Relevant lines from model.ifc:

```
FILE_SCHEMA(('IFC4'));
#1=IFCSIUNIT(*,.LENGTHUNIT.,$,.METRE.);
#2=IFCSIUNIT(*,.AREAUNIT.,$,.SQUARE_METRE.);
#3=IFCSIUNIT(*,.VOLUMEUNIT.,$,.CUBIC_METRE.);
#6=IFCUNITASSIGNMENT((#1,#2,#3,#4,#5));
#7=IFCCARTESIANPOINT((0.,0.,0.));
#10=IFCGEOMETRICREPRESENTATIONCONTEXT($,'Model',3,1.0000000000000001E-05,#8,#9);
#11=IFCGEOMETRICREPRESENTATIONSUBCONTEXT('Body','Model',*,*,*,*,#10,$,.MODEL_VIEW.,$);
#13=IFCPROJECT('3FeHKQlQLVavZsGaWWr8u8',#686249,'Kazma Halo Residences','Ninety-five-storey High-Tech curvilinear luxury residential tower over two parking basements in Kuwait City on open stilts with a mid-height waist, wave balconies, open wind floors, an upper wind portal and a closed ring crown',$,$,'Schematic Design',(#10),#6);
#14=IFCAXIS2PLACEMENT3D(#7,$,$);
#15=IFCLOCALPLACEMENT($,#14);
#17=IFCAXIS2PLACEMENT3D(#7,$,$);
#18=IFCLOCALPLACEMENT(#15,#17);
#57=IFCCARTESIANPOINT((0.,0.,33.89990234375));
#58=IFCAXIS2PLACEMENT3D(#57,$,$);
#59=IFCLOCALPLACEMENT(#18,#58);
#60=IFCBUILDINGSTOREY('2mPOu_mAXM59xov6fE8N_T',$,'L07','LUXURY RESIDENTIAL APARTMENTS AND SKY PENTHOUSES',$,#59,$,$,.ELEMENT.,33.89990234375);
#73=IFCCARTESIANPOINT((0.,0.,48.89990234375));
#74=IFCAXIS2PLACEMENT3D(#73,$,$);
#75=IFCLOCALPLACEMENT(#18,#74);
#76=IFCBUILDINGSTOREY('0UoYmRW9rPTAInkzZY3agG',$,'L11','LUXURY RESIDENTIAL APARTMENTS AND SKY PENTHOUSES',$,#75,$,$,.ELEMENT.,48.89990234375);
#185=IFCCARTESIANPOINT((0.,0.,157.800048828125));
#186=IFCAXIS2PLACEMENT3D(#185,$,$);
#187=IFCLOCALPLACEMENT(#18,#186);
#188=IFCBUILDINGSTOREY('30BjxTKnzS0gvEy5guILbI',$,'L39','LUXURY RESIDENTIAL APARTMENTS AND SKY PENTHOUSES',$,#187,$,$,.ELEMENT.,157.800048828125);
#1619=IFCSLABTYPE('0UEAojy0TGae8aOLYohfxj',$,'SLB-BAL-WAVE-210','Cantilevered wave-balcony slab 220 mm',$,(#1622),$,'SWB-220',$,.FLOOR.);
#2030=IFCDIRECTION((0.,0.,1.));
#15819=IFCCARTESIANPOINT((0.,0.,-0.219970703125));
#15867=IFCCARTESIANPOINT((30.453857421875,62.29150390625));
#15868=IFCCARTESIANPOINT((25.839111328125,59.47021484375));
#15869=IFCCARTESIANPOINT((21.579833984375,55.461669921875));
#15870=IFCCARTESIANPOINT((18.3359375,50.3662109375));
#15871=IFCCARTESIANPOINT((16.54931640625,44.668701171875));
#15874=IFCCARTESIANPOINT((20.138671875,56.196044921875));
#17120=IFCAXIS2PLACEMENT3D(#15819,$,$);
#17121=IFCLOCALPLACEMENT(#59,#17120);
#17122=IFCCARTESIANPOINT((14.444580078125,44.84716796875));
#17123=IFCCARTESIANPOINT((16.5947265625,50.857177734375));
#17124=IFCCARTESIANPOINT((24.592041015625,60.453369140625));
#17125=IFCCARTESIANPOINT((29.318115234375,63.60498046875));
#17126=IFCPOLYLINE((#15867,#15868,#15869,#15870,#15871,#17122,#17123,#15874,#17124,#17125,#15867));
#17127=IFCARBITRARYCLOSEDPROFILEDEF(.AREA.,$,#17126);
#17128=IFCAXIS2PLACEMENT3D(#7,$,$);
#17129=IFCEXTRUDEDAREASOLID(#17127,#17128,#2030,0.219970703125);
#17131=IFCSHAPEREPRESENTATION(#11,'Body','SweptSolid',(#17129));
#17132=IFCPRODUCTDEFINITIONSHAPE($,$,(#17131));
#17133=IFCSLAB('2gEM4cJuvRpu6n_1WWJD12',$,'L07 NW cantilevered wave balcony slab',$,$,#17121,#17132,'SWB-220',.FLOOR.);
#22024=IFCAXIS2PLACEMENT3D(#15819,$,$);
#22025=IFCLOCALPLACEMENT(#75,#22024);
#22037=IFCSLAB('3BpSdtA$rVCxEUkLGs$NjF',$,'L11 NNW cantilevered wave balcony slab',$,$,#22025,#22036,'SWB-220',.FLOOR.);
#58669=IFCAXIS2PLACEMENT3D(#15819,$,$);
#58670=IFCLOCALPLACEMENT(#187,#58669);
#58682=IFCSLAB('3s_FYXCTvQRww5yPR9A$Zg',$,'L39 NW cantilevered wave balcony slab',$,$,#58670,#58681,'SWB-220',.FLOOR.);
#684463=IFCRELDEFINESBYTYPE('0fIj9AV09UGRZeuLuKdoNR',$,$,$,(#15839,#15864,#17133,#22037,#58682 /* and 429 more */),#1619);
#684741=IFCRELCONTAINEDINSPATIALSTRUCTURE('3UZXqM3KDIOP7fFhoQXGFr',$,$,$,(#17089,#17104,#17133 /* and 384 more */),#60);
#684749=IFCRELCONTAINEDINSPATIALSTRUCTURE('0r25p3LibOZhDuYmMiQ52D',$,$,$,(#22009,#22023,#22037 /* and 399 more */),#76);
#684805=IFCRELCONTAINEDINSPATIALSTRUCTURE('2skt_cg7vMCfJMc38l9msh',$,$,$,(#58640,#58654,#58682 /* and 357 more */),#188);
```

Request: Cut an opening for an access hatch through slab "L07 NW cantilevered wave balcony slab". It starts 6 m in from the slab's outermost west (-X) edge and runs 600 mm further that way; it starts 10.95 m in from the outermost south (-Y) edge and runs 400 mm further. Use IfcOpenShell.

```python
import numpy as np
import ifcopenshell
import ifcopenshell.api.feature
import ifcopenshell.api.geometry
import ifcopenshell.api.root
import ifcopenshell.geom
import ifcopenshell.util.placement
import ifcopenshell.util.representation
import ifcopenshell.util.shape
import ifcopenshell.util.unit

model = ifcopenshell.open("model.ifc")
unit_scale = ifcopenshell.util.unit.calculate_unit_scale(model)
settings = ifcopenshell.geom.settings()


def volume(element):
    """Net volume in cubic metres, openings subtracted."""
    shape = ifcopenshell.geom.create_shape(settings, element)
    return ifcopenshell.util.shape.get_volume(shape.geometry)


slab = model.by_id(17133)
before = volume(slab)

# Extent in the slab's own axes, in metres. The edges named are its -X and -Y sides.
slab_shape = ifcopenshell.geom.create_shape(settings, slab)
vertices = ifcopenshell.util.shape.get_vertices(slab_shape.geometry)
x_min, y_min, bottom = vertices.min(axis=0)
top = vertices[:, 2].max()

opening = ifcopenshell.api.root.create_entity(model, ifc_class="IfcOpeningElement", name="Access hatch opening", predefined_type="OPENING")
context = ifcopenshell.util.representation.get_context(model, "Model", "Body", "MODEL_VIEW")
width, depth = 0.6, 0.4
outline = [(0.0, 0.0), (width, 0.0), (width, depth), (0.0, depth), (0.0, 0.0)]
# Overshoot both faces by 50 mm so the cut is clean.
shape = ifcopenshell.api.geometry.add_slab_representation(
    model, context=context, depth=top - bottom + 0.1, polyline=outline
)
ifcopenshell.api.geometry.assign_representation(model, product=opening, representation=shape)

matrix = ifcopenshell.util.placement.get_local_placement(slab.ObjectPlacement)
matrix[:, 3] = matrix @ np.append(np.array([x_min + 6, y_min + 10.95, bottom - 0.05]) / unit_scale, 1.0)
ifcopenshell.api.geometry.edit_object_placement(model, product=opening, matrix=matrix, is_si=False)
ifcopenshell.api.feature.add_feature(model, feature=opening, element=slab)

after = volume(slab)

print(f"slab volume {before:.3f} -> {after:.3f} m3")

model.write("model_edited.ifc")
```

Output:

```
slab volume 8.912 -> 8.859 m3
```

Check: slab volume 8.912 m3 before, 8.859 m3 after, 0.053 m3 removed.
